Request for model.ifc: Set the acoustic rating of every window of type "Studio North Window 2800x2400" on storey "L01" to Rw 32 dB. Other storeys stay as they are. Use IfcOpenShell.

First a look at what the model holds.

```python
import ifcopenshell
import ifcopenshell.util.element

model = ifcopenshell.open("model.ifc")
print(model.schema)
storey = next(s for s in model.by_type("IfcBuildingStorey") if s.Name == "L01")
windows = [e for e in ifcopenshell.util.element.get_decomposition(storey) if e.is_a("IfcWindow")]
seen = {}
for e in windows:
    element_type = ifcopenshell.util.element.get_type(e)
    key = (element_type.Name if element_type != e and element_type else None, ifcopenshell.util.element.get_pset(e, "Pset_WindowCommon", "AcousticRating"))
    seen[key] = seen.get(key, 0) + 1
for (name, value), count in sorted(seen.items(), key=str):
    print(count, "x", name, "|", value)
```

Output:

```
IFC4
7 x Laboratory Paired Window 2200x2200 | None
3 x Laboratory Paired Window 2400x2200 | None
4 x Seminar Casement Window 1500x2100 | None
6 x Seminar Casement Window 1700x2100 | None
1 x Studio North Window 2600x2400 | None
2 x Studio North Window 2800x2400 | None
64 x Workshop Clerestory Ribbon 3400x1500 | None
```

```python
import ifcopenshell
import ifcopenshell.api.pset
import ifcopenshell.util.element

model = ifcopenshell.open("model.ifc")

storey = next(s for s in model.by_type("IfcBuildingStorey") if s.Name == "L01")
windows = [e for e in ifcopenshell.util.element.get_decomposition(storey) if e.is_a("IfcWindow")]

count = 0
for e in windows:
    element_type = ifcopenshell.util.element.get_type(e)
    if element_type in (None, e) or element_type.Name != "Studio North Window 2800x2400":
        continue
    # add_pset returns the element's existing set when there is one.
    pset = ifcopenshell.api.pset.add_pset(model, product=e, name="Pset_WindowCommon")
    ifcopenshell.api.pset.edit_pset(model, pset=pset, properties={"AcousticRating": "Rw 32 dB"})
    count += 1

print(count, "windows updated")

model.write("model_updated.ifc")
```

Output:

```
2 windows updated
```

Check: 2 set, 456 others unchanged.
